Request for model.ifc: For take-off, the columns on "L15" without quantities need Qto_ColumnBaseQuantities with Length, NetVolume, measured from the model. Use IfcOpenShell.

First a look at what the model holds.

```python
import ifcopenshell
import ifcopenshell.util.element
import ifcopenshell.util.unit

model = ifcopenshell.open("model.ifc")
print(model.schema)
for unit_type in ("LENGTHUNIT", "AREAUNIT", "VOLUMEUNIT"):
    print(unit_type, ifcopenshell.util.unit.calculate_unit_scale(model, unit_type))
storey = next(s for s in model.by_type("IfcBuildingStorey") if s.Name == "L15")
columns = [e for e in ifcopenshell.util.element.get_decomposition(storey) if e.is_a("IfcColumn")]
for e in sorted(columns, key=lambda e: e.id()):
    print(e.id(), e.is_a(), e.Name, list(ifcopenshell.util.element.get_psets(e, qtos_only=True)), sep=" | ")
```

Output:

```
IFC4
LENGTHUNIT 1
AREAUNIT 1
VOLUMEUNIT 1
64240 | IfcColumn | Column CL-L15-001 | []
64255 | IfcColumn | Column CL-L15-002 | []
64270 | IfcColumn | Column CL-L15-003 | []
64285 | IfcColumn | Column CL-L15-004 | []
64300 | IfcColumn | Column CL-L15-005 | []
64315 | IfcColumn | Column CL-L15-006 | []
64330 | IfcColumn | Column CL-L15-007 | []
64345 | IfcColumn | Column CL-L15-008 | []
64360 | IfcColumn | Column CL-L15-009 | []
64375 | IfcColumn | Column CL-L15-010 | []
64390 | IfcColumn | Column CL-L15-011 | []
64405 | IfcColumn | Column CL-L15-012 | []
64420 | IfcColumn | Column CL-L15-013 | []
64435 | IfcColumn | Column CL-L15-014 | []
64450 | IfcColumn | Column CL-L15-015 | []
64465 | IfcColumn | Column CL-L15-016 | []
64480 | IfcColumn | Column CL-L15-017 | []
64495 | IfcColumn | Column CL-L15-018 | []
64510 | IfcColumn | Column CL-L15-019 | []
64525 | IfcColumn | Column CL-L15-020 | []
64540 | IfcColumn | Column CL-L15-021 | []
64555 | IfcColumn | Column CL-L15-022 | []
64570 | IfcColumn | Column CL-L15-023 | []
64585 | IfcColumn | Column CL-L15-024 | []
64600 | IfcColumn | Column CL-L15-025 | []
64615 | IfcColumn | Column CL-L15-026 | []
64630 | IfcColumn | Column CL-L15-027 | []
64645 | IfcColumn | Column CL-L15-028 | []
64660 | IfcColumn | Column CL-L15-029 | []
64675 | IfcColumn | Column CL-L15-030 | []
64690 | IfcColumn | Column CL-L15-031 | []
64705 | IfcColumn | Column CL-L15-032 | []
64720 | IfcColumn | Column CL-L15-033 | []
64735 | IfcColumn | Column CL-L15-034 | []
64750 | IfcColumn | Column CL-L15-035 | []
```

```python
import ifcopenshell
import ifcopenshell.api.pset
import ifcopenshell.geom
import ifcopenshell.util.element
import ifcopenshell.util.shape
import ifcopenshell.util.unit

model = ifcopenshell.open("model.ifc")
unit_scale = ifcopenshell.util.unit.calculate_unit_scale(model)
volume_scale = ifcopenshell.util.unit.calculate_unit_scale(model, "VOLUMEUNIT")
settings = ifcopenshell.geom.settings()

storey = next(s for s in model.by_type("IfcBuildingStorey") if s.Name == "L15")
columns = [e for e in ifcopenshell.util.element.get_decomposition(storey) if e.is_a("IfcColumn")]

for e in sorted(columns, key=lambda e: e.id()):
    if ifcopenshell.util.element.get_psets(e, qtos_only=True, should_inherit=False):
        continue
    # Geometry comes back in metres, in the element's own axes.
    shape = ifcopenshell.geom.create_shape(settings, e)
    values = {
        "Length": ifcopenshell.util.shape.get_z(shape.geometry) / unit_scale,
        "NetVolume": ifcopenshell.util.shape.get_volume(shape.geometry) / volume_scale,
    }
    qto = ifcopenshell.api.pset.add_qto(model, product=e, name="Qto_ColumnBaseQuantities")
    ifcopenshell.api.pset.edit_qto(model, qto=qto, properties=values)
    print(e.id(), {k: round(v, 3) for k, v in values.items()})

model.write("model-out.ifc")
```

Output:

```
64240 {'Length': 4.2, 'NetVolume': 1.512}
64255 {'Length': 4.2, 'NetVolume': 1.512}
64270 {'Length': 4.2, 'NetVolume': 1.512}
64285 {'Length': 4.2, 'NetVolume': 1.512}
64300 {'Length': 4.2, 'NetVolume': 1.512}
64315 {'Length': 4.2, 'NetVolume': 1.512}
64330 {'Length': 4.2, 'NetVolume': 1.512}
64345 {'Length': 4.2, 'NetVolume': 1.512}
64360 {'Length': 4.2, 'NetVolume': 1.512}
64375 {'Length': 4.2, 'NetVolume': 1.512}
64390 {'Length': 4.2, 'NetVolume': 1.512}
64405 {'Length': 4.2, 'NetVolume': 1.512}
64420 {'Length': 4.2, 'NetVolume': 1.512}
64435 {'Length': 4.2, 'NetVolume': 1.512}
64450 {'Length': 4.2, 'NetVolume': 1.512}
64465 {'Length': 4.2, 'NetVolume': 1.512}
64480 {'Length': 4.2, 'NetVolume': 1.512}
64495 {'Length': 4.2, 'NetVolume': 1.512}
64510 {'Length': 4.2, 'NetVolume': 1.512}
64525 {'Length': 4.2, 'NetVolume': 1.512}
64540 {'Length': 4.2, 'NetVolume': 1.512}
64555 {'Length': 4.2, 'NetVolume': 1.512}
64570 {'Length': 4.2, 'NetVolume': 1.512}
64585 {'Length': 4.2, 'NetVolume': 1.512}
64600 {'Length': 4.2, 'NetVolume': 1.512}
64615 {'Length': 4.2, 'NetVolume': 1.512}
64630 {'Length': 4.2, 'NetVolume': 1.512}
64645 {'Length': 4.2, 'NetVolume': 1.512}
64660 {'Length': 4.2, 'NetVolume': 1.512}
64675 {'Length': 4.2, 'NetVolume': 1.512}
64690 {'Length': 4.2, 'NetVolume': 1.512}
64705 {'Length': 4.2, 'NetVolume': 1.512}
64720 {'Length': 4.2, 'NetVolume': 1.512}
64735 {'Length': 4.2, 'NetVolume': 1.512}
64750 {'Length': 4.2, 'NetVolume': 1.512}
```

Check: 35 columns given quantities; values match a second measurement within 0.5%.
